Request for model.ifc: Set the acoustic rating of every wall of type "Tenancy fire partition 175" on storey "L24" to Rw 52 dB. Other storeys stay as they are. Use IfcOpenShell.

First a look at what the model holds.

```python
import ifcopenshell
import ifcopenshell.util.element

model = ifcopenshell.open("model.ifc")
print(model.schema)
storey = next(s for s in model.by_type("IfcBuildingStorey") if s.Name == "L24")
walls = [e for e in ifcopenshell.util.element.get_decomposition(storey) if e.is_a("IfcWall")]
seen = {}
for e in walls:
    element_type = ifcopenshell.util.element.get_type(e)
    key = (element_type.Name if element_type != e and element_type else None, ifcopenshell.util.element.get_pset(e, "Pset_WallCommon", "AcousticRating"))
    seen[key] = seen.get(key, 0) + 1
for (name, value), count in sorted(seen.items(), key=str):
    print(count, "x", name, "|", value)
```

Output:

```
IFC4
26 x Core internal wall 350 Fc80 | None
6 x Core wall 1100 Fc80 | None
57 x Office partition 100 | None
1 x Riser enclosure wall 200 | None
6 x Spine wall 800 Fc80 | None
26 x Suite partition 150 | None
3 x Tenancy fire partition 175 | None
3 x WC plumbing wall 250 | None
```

```python
import ifcopenshell
import ifcopenshell.api.pset
import ifcopenshell.util.element

model = ifcopenshell.open("model.ifc")

storey = next(s for s in model.by_type("IfcBuildingStorey") if s.Name == "L24")
walls = [e for e in ifcopenshell.util.element.get_decomposition(storey) if e.is_a("IfcWall")]

count = 0
for e in walls:
    element_type = ifcopenshell.util.element.get_type(e)
    if element_type in (None, e) or element_type.Name != "Tenancy fire partition 175":
        continue
    found = ifcopenshell.util.element.get_pset(e, "Pset_WallCommon", should_inherit=False)
    if found:
        pset = model.by_id(found["id"])
        if len(ifcopenshell.util.element.get_elements_by_pset(pset)) > 1:
            pset = ifcopenshell.api.pset.unshare_pset(model, products=[e], pset=pset)[0]
    else:
        pset = ifcopenshell.api.pset.add_pset(model, product=e, name="Pset_WallCommon")
    ifcopenshell.api.pset.edit_pset(model, pset=pset, properties={"AcousticRating": "Rw 52 dB"})
    count += 1

print(count, "walls updated")

model.write("model_v2.ifc")
```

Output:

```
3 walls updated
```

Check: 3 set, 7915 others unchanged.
